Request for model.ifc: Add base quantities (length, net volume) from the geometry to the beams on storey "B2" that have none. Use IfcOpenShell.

First a look at what the model holds.

```python
import ifcopenshell
import ifcopenshell.util.element
import ifcopenshell.util.unit

model = ifcopenshell.open("model.ifc")
print(model.schema)
for unit_type in ("LENGTHUNIT", "AREAUNIT", "VOLUMEUNIT"):
    print(unit_type, ifcopenshell.util.unit.calculate_unit_scale(model, unit_type))
storey = next(s for s in model.by_type("IfcBuildingStorey") if s.Name == "B2")
beams = [e for e in ifcopenshell.util.element.get_decomposition(storey) if e.is_a("IfcBeam")]
for e in sorted(beams, key=lambda e: e.id()):
    print(e.id(), e.is_a(), e.Name, list(ifcopenshell.util.element.get_psets(e, qtos_only=True)), sep=" | ")
```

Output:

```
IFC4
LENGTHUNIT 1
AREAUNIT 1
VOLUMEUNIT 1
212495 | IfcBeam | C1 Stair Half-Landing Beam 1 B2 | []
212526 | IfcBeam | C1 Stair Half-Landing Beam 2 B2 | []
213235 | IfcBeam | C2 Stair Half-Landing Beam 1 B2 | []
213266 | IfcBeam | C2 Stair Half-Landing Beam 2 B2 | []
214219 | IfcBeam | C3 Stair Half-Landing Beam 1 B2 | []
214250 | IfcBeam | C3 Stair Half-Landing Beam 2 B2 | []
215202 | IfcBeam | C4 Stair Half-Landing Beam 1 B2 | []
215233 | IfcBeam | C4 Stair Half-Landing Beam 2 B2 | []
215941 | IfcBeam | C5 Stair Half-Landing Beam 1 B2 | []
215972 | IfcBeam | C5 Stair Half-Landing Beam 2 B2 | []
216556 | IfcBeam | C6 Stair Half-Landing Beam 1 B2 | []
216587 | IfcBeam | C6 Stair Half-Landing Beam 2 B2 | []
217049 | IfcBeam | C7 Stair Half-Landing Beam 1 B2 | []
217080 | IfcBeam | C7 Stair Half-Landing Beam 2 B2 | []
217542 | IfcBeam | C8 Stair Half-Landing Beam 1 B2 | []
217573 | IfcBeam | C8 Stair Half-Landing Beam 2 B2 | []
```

```python
import ifcopenshell
import ifcopenshell.api.pset
import ifcopenshell.geom
import ifcopenshell.util.element
import ifcopenshell.util.shape
import ifcopenshell.util.unit

model = ifcopenshell.open("model.ifc")
unit_scale = ifcopenshell.util.unit.calculate_unit_scale(model)
volume_scale = ifcopenshell.util.unit.calculate_unit_scale(model, "VOLUMEUNIT")
settings = ifcopenshell.geom.settings()

storey = next(s for s in model.by_type("IfcBuildingStorey") if s.Name == "B2")
beams = [e for e in ifcopenshell.util.element.get_decomposition(storey) if e.is_a("IfcBeam")]

for e in sorted(beams, key=lambda e: e.id()):
    if ifcopenshell.util.element.get_psets(e, qtos_only=True, should_inherit=False):
        continue
    # Geometry comes back in metres, in the element's own axes.
    shape = ifcopenshell.geom.create_shape(settings, e)
    values = {
        "Length": ifcopenshell.util.shape.get_max_xyz(shape.geometry) / unit_scale,
        "NetVolume": ifcopenshell.util.shape.get_volume(shape.geometry) / volume_scale,
    }
    qto = ifcopenshell.api.pset.add_qto(model, product=e, name="Qto_BeamBaseQuantities")
    ifcopenshell.api.pset.edit_qto(model, qto=qto, properties=values)
    print(e.id(), {k: round(v, 3) for k, v in values.items()})

model.write("model-out.ifc")
```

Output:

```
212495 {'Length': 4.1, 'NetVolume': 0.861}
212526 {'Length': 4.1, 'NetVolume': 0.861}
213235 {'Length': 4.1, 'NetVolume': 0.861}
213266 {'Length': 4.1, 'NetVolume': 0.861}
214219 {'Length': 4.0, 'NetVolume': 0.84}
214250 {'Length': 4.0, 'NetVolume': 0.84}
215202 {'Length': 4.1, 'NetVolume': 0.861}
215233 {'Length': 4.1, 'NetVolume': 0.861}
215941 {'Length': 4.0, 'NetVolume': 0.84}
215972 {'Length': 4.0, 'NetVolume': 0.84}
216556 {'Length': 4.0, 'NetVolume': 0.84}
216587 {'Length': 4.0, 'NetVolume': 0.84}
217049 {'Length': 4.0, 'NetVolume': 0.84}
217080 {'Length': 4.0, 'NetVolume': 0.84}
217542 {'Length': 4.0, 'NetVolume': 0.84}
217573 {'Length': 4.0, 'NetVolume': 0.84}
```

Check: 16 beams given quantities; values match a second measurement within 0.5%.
